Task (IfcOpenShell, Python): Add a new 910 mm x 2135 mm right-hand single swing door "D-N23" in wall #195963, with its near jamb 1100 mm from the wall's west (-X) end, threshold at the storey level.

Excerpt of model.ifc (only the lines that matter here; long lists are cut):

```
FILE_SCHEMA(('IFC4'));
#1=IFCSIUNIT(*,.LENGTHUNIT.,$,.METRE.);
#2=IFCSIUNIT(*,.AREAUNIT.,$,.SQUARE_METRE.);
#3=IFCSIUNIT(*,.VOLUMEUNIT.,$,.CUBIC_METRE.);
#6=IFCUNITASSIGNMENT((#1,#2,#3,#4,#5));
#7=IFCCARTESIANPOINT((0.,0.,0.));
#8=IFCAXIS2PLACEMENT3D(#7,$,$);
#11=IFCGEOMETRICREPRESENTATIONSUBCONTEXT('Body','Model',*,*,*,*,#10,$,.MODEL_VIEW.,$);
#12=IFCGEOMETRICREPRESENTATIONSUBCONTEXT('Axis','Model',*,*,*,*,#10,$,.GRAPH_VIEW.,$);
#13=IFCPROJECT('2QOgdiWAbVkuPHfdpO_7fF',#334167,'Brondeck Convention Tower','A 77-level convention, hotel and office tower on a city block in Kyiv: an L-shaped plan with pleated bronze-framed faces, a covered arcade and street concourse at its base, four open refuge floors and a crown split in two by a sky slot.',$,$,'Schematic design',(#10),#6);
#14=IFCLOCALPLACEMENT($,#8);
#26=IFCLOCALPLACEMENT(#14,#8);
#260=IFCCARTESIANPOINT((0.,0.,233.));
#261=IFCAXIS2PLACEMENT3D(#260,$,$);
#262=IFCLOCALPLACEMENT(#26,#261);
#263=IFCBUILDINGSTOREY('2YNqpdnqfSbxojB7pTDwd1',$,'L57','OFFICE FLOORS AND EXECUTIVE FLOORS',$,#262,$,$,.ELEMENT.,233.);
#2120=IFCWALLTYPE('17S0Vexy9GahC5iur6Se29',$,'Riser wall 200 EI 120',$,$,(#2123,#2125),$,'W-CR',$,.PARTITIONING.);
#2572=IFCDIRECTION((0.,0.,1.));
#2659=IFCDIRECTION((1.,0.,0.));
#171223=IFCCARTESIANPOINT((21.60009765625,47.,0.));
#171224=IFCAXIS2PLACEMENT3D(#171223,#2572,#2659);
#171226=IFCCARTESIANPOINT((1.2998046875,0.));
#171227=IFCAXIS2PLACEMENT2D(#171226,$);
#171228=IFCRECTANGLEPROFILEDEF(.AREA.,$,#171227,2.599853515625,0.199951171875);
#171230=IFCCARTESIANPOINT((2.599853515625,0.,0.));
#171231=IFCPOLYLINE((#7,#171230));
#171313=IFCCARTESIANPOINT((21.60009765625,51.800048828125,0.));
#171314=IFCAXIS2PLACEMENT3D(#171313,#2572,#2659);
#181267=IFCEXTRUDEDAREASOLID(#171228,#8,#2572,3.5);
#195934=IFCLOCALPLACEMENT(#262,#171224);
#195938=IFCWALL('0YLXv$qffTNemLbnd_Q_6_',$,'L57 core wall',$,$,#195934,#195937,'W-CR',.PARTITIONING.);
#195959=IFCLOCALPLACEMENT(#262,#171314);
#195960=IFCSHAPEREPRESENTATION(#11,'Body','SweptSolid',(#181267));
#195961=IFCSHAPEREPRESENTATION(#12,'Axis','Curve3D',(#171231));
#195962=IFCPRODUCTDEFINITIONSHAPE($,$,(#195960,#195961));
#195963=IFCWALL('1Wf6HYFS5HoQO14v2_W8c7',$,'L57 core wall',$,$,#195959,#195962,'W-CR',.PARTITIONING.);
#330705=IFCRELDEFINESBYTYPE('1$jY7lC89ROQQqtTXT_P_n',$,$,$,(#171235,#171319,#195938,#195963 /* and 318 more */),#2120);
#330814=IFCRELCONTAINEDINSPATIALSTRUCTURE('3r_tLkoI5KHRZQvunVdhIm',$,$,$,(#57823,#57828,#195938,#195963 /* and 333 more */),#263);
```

```python
import numpy as np
import ifcopenshell
import ifcopenshell.api.feature
import ifcopenshell.api.geometry
import ifcopenshell.api.root
import ifcopenshell.api.spatial
import ifcopenshell.geom
import ifcopenshell.util.element
import ifcopenshell.util.placement
import ifcopenshell.util.representation
import ifcopenshell.util.shape
import ifcopenshell.util.unit

model = ifcopenshell.open("model.ifc")
unit_scale = ifcopenshell.util.unit.calculate_unit_scale(model)
settings = ifcopenshell.geom.settings()


def volume(element):
    """Net volume in cubic metres, openings subtracted."""
    shape = ifcopenshell.geom.create_shape(settings, element)
    return ifcopenshell.util.shape.get_volume(shape.geometry)


wall = model.by_id(195963)
storey = ifcopenshell.util.element.get_container(wall, ifc_class="IfcBuildingStorey")
context = ifcopenshell.util.representation.get_context(model, "Model", "Body", "MODEL_VIEW")
before = volume(wall)

width, height, from_end, sill = 0.91, 2.135, 1.1, 0.0  # metres

# The wall runs along its own X axis, and the end named is its -X end.
wall_shape = ifcopenshell.geom.create_shape(settings, wall)
x, y, z = ifcopenshell.util.shape.get_vertices(wall_shape.geometry).T
start = x.min() + from_end
face, thickness = float(y.min()), float(y.max() - y.min())
wall_matrix = ifcopenshell.util.placement.get_local_placement(wall.ObjectPlacement)
level = ifcopenshell.util.placement.get_local_placement(storey.ObjectPlacement)[2, 3]


def in_wall(x, y):
    """Placement at x, y metres in the wall's axes, at sill height."""
    matrix = wall_matrix.copy()
    matrix[:, 3] = wall_matrix @ np.array([x / unit_scale, y / unit_scale, 0.0, 1.0])
    matrix[2, 3] = level + sill / unit_scale
    return matrix


# Opening: a box that overshoots both wall faces by 50 mm.
opening = ifcopenshell.api.root.create_entity(model, ifc_class="IfcOpeningElement", predefined_type="OPENING")
box = ifcopenshell.api.geometry.add_wall_representation(
    model, context=context, length=width, height=height, thickness=thickness + 0.1
)
ifcopenshell.api.geometry.assign_representation(model, product=opening, representation=box)
ifcopenshell.api.geometry.edit_object_placement(model, product=opening, matrix=in_wall(start, face - 0.05), is_si=False)
ifcopenshell.api.feature.add_feature(model, feature=opening, element=wall)

door = ifcopenshell.api.root.create_entity(model, ifc_class="IfcDoor", name="D-N23", predefined_type="DOOR")
door.OverallWidth, door.OverallHeight = width / unit_scale, height / unit_scale
door.OperationType = "SINGLE_SWING_RIGHT"
body = ifcopenshell.api.geometry.add_door_representation(
    model,
    context=context,
    overall_width=door.OverallWidth,
    overall_height=door.OverallHeight,
    operation_type="SINGLE_SWING_RIGHT",
    lining_properties={"LiningDepth": thickness / unit_scale, "ThresholdDepth": thickness / unit_scale},
)
ifcopenshell.api.geometry.assign_representation(model, product=door, representation=body)
ifcopenshell.api.spatial.assign_container(model, products=[door], relating_structure=storey)
ifcopenshell.api.feature.add_filling(model, opening=opening, element=door)

# The lining spans the wall, so the door starts at the wall face.
ifcopenshell.api.geometry.edit_object_placement(model, product=door, matrix=in_wall(start, face), is_si=False)

after = volume(wall)

print(f"wall volume {before:.3f} -> {after:.3f} m3")

model.write("model_edited.ifc")
```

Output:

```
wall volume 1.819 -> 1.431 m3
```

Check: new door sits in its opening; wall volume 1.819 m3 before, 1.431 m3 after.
